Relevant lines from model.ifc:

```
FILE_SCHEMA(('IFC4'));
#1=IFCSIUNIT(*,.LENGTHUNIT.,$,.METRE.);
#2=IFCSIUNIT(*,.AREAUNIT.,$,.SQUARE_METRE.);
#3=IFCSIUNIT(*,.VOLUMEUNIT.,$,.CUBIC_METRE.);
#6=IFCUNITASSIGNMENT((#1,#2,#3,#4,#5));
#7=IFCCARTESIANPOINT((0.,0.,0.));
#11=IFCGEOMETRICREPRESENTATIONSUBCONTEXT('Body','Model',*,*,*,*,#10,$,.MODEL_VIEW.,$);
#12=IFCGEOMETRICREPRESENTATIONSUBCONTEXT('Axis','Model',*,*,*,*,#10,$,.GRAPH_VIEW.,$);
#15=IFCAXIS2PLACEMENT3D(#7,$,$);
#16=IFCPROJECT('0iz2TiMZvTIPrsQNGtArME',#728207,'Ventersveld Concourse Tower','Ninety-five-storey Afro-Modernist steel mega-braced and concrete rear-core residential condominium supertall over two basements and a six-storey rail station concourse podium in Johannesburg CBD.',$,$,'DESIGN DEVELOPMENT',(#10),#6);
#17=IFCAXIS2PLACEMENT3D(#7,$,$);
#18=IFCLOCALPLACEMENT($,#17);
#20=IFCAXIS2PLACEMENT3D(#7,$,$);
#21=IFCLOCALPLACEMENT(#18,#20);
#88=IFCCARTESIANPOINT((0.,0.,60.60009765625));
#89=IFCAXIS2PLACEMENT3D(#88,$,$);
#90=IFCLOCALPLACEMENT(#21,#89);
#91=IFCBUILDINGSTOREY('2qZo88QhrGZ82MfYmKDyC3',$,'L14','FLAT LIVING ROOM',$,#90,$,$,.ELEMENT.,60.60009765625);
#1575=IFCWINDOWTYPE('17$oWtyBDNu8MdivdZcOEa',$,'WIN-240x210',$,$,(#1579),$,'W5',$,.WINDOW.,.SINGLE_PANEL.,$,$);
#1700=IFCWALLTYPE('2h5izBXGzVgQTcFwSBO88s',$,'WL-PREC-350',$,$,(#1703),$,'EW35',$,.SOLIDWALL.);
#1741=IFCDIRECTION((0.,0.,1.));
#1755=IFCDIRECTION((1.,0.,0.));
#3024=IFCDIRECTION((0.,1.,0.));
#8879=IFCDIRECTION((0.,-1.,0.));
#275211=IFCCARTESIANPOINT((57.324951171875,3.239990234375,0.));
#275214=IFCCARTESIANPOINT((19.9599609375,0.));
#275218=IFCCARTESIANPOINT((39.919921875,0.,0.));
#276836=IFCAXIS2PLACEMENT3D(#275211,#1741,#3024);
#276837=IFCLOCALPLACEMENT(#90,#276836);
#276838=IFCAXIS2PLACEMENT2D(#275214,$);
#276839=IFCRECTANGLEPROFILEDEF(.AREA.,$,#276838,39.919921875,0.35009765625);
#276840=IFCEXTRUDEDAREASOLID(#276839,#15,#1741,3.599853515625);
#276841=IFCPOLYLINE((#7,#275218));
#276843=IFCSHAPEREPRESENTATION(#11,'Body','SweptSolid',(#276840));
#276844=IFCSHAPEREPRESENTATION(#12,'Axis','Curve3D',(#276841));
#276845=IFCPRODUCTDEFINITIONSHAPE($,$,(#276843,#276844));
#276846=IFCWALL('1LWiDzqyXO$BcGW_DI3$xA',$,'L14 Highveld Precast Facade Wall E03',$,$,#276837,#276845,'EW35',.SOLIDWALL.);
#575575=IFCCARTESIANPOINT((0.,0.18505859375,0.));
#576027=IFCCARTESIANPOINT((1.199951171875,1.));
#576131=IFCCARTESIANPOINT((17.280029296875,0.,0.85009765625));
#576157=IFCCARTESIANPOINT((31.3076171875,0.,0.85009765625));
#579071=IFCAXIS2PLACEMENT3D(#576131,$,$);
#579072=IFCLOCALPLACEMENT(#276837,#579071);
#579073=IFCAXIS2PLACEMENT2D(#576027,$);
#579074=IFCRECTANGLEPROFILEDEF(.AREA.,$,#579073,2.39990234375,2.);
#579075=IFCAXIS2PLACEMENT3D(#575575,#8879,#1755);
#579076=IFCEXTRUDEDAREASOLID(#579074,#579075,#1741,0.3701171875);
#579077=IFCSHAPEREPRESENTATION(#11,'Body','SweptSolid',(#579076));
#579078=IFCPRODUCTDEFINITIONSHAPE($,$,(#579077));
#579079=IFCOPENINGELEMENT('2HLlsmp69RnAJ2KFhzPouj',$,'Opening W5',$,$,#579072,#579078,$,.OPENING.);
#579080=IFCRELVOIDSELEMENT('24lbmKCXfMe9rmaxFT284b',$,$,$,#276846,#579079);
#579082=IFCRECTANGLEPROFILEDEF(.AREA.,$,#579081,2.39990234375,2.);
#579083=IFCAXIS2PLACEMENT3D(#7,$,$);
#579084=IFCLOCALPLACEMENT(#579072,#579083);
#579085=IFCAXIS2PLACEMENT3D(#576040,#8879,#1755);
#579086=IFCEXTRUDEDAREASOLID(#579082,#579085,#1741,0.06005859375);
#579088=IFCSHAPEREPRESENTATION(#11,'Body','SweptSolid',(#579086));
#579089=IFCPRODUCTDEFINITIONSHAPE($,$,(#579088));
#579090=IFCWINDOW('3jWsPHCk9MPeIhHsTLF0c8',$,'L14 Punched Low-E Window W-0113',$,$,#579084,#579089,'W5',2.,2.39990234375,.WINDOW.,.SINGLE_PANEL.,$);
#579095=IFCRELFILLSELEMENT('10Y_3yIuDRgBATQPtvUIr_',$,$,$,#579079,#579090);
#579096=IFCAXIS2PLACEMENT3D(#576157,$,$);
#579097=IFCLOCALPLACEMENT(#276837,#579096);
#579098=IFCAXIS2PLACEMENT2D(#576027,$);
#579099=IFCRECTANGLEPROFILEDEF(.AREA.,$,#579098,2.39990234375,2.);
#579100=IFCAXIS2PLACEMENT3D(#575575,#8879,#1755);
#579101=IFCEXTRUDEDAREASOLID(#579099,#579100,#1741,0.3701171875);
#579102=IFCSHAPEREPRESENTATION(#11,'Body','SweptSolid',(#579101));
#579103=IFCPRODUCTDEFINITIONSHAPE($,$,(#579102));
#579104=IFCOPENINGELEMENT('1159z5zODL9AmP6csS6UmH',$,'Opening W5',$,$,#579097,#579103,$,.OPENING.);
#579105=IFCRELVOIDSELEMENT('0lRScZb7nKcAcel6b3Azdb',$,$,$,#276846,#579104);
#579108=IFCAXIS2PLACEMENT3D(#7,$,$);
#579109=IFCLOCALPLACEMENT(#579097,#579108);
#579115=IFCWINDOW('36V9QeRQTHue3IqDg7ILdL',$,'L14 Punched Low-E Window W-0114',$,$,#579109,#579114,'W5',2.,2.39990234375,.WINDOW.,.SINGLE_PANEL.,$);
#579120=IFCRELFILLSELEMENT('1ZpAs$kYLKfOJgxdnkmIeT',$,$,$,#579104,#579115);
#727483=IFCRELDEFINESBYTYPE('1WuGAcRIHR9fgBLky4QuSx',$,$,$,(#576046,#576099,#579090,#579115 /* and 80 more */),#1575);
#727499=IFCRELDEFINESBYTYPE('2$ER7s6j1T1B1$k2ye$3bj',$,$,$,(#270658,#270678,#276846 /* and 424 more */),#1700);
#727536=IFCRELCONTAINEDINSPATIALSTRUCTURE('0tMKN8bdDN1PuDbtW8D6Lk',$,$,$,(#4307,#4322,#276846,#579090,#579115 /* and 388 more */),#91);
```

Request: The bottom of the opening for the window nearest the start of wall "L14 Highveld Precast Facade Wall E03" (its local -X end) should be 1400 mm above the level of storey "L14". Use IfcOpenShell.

```python
import numpy as np
import ifcopenshell
import ifcopenshell.api.geometry
import ifcopenshell.geom
import ifcopenshell.util.element
import ifcopenshell.util.placement
import ifcopenshell.util.shape
import ifcopenshell.util.unit

model = ifcopenshell.open("model.ifc")
unit_scale = ifcopenshell.util.unit.calculate_unit_scale(model)

window = model.by_guid("3jWsPHCk9MPeIhHsTLF0c8")
opening = window.FillsVoids[0].RelatingOpeningElement
storey = ifcopenshell.util.element.get_container(window, ifc_class="IfcBuildingStorey")
level = ifcopenshell.util.placement.get_local_placement(storey.ObjectPlacement)[2, 3]

# The opening's origin need not be at the sill, so measure its lowest point.
shape = ifcopenshell.geom.create_shape(ifcopenshell.geom.settings(), opening)
bottom = ifcopenshell.util.shape.get_shape_bottom_elevation(shape, shape.geometry) / unit_scale
dz = level + 1.4 / unit_scale - bottom

shift = np.array([0.0, 0.0, dz])
# The window is placed relative to its opening, so it follows when the opening moves.
matrix = ifcopenshell.util.placement.get_local_placement(opening.ObjectPlacement)
matrix[:3, 3] += shift
ifcopenshell.api.geometry.edit_object_placement(
    model, product=opening, matrix=matrix, is_si=False, should_transform_children=True
)

print(f"moved by {dz * unit_scale:+.3f} m")

model.write("model_rev.ifc")
```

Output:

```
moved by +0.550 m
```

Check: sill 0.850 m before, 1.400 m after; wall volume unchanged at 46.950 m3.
